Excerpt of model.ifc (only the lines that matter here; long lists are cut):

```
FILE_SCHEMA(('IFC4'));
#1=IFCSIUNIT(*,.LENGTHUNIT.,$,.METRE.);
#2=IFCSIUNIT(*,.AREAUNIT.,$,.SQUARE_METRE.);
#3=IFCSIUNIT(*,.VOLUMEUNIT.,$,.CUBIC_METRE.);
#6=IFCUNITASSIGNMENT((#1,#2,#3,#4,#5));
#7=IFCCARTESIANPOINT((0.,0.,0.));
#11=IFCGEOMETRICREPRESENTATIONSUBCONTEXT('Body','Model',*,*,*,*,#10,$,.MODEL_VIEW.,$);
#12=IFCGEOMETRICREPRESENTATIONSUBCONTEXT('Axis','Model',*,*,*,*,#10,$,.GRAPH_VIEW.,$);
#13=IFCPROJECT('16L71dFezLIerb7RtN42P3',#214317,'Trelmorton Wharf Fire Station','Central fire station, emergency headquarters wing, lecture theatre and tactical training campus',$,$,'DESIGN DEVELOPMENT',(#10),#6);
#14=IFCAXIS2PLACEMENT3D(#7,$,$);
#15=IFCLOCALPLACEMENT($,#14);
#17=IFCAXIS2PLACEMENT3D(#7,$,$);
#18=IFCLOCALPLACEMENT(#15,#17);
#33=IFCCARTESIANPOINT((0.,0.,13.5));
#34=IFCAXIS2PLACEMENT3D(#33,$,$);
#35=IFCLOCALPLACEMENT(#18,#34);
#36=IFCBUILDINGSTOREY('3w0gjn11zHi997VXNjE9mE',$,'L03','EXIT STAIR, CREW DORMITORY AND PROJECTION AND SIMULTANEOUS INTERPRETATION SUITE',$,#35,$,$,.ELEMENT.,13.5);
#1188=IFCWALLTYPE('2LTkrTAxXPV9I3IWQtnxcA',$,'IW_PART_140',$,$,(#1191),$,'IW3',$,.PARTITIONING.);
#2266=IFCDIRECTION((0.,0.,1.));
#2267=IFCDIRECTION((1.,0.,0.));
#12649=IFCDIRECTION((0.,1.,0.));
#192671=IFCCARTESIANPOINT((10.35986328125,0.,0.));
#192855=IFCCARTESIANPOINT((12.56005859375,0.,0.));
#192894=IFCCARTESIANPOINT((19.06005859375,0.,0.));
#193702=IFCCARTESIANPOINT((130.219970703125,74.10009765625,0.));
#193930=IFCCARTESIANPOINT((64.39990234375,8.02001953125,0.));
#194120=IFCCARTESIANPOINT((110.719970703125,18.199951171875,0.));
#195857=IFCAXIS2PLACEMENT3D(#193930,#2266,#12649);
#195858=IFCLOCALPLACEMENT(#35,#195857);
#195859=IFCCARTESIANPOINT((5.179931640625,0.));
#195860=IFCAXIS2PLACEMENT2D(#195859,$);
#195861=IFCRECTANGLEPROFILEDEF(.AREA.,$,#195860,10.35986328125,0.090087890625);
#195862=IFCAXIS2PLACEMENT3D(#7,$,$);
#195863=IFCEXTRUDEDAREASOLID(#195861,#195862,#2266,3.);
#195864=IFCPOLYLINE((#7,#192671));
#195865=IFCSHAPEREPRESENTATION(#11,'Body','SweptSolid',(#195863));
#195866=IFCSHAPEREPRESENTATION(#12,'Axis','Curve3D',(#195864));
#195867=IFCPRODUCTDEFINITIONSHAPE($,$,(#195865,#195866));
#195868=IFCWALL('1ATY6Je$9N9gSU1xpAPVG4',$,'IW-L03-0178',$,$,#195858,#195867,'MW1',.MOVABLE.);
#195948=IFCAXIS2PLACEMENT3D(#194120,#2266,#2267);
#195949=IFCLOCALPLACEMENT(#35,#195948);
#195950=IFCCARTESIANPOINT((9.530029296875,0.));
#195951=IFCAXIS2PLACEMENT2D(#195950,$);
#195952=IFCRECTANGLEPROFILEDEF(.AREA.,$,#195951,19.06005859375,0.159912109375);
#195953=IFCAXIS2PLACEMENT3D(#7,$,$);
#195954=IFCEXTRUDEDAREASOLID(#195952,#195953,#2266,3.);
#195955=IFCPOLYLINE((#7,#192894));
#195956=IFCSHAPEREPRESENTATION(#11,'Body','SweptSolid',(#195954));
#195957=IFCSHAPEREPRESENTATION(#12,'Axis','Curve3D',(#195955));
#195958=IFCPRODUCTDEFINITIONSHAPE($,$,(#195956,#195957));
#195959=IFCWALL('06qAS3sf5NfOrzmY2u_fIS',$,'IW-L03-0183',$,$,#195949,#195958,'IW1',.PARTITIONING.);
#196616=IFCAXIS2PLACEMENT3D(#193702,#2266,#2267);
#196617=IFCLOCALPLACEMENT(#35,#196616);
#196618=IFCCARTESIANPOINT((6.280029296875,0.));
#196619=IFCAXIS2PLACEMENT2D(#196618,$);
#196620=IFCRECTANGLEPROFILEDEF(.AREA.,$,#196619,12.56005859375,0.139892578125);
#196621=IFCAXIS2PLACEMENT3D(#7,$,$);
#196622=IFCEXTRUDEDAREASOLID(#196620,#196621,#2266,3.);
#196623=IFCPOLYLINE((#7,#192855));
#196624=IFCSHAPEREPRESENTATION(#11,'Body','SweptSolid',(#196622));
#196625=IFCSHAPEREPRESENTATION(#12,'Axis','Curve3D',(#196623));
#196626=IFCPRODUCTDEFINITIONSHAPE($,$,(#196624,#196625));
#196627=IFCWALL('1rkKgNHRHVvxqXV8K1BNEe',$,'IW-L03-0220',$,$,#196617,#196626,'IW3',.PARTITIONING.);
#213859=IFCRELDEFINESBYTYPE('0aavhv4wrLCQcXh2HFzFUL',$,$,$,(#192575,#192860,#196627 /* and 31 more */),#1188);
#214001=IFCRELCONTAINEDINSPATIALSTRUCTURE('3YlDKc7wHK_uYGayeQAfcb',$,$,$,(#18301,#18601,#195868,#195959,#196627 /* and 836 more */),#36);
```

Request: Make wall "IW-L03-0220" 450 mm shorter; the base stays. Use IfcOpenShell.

```python
import ifcopenshell
import ifcopenshell.geom
import ifcopenshell.util.representation
import ifcopenshell.util.shape

model = ifcopenshell.open("model.ifc")
settings = ifcopenshell.geom.settings()


def volume(element):
    """Net volume in cubic metres, openings subtracted."""
    shape = ifcopenshell.geom.create_shape(settings, element)
    return ifcopenshell.util.shape.get_volume(shape.geometry)


wall = model.by_id(196627)
before = volume(wall)

body = ifcopenshell.util.representation.get_representation(wall, "Model", "Body")
solid = body.Items[0]
old_height = solid.Depth
solid.Depth -= 0.45
after = volume(wall)

print(f"height {old_height:g} -> {solid.Depth:g}, volume {before:.3f} -> {after:.3f} m3")

model.write("model_v2.ifc")
```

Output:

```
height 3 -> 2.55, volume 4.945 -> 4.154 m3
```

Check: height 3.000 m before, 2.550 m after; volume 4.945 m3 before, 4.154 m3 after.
